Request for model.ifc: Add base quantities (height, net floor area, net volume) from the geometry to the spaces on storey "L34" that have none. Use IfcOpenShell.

First a look at what the model holds.

```python
import ifcopenshell
import ifcopenshell.util.element
import ifcopenshell.util.unit

model = ifcopenshell.open("model.ifc")
print(model.schema)
for unit_type in ("LENGTHUNIT", "AREAUNIT", "VOLUMEUNIT"):
    print(unit_type, ifcopenshell.util.unit.calculate_unit_scale(model, unit_type))
storey = next(s for s in model.by_type("IfcBuildingStorey") if s.Name == "L34")
spaces = [e for e in ifcopenshell.util.element.get_decomposition(storey) if e.is_a("IfcSpace")]
for e in sorted(spaces, key=lambda e: e.id()):
    print(e.id(), e.is_a(), e.Name, list(ifcopenshell.util.element.get_psets(e, qtos_only=True)), sep=" | ")
```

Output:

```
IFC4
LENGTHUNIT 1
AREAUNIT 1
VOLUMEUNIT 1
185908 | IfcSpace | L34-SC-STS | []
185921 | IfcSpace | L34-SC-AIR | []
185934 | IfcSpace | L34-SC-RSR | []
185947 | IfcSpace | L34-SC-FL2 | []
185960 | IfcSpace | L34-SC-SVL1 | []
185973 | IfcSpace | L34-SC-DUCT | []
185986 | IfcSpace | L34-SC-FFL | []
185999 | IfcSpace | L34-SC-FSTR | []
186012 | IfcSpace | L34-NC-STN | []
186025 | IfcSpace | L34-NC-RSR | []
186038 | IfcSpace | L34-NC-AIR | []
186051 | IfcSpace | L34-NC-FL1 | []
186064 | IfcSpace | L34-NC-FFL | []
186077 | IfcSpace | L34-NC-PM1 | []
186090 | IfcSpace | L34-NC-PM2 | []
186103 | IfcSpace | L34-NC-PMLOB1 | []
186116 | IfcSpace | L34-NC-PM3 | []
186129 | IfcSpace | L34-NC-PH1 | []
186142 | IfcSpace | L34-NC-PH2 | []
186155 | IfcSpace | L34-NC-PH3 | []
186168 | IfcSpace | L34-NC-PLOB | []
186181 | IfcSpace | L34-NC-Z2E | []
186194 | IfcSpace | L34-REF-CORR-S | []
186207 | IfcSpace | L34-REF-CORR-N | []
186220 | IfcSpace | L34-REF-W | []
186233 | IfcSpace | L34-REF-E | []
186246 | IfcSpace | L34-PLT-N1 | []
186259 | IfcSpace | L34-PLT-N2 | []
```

```python
import ifcopenshell
import ifcopenshell.api.pset
import ifcopenshell.geom
import ifcopenshell.util.element
import ifcopenshell.util.shape
import ifcopenshell.util.unit

model = ifcopenshell.open("model.ifc")
unit_scale = ifcopenshell.util.unit.calculate_unit_scale(model)
area_scale = ifcopenshell.util.unit.calculate_unit_scale(model, "AREAUNIT")
volume_scale = ifcopenshell.util.unit.calculate_unit_scale(model, "VOLUMEUNIT")
settings = ifcopenshell.geom.settings()

storey = next(s for s in model.by_type("IfcBuildingStorey") if s.Name == "L34")
spaces = [e for e in ifcopenshell.util.element.get_decomposition(storey) if e.is_a("IfcSpace")]

for e in sorted(spaces, key=lambda e: e.id()):
    if ifcopenshell.util.element.get_psets(e, qtos_only=True, should_inherit=False):
        continue
    # Geometry comes back in metres, in the element's own axes.
    shape = ifcopenshell.geom.create_shape(settings, e)
    values = {
        "Height": ifcopenshell.util.shape.get_z(shape.geometry) / unit_scale,
        "NetFloorArea": ifcopenshell.util.shape.get_footprint_area(shape.geometry) / area_scale,
        "NetVolume": ifcopenshell.util.shape.get_volume(shape.geometry) / volume_scale,
    }
    qto = ifcopenshell.api.pset.add_qto(model, product=e, name="Qto_SpaceBaseQuantities")
    ifcopenshell.api.pset.edit_qto(model, qto=qto, properties=values)
    print(e.id(), {k: round(v, 3) for k, v in values.items()})

model.write("model_updated.ifc")
```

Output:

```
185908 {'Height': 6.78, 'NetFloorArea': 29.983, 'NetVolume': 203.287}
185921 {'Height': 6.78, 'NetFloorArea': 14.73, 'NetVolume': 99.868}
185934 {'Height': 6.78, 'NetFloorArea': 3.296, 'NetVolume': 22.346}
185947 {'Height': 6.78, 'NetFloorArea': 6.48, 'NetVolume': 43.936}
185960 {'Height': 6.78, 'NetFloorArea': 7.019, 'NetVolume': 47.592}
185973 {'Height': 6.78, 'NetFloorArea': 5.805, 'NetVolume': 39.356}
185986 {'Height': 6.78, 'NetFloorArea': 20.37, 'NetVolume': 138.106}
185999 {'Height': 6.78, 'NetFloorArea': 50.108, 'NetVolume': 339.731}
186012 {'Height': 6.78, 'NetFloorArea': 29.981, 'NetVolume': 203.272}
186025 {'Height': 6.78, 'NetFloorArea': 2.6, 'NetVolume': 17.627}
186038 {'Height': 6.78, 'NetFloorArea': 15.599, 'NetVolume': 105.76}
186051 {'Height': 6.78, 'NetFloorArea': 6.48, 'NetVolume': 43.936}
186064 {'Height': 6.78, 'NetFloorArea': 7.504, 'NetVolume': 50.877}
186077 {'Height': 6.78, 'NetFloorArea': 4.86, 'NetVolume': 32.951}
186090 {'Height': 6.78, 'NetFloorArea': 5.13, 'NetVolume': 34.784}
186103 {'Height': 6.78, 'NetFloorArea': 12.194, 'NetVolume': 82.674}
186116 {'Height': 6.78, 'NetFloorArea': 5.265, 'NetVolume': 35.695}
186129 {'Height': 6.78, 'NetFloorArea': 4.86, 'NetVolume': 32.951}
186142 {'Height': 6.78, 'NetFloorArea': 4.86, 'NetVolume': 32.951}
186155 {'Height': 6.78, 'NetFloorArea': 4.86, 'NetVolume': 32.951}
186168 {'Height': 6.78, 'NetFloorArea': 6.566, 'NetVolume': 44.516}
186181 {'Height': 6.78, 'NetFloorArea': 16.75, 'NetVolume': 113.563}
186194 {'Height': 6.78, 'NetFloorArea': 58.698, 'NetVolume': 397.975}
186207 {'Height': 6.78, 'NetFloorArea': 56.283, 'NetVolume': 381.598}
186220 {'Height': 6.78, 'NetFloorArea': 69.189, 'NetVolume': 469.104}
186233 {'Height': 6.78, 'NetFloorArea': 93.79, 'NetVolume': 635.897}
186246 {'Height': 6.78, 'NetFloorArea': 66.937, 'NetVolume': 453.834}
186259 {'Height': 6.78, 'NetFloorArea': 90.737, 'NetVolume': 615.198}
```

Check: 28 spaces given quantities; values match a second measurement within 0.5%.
